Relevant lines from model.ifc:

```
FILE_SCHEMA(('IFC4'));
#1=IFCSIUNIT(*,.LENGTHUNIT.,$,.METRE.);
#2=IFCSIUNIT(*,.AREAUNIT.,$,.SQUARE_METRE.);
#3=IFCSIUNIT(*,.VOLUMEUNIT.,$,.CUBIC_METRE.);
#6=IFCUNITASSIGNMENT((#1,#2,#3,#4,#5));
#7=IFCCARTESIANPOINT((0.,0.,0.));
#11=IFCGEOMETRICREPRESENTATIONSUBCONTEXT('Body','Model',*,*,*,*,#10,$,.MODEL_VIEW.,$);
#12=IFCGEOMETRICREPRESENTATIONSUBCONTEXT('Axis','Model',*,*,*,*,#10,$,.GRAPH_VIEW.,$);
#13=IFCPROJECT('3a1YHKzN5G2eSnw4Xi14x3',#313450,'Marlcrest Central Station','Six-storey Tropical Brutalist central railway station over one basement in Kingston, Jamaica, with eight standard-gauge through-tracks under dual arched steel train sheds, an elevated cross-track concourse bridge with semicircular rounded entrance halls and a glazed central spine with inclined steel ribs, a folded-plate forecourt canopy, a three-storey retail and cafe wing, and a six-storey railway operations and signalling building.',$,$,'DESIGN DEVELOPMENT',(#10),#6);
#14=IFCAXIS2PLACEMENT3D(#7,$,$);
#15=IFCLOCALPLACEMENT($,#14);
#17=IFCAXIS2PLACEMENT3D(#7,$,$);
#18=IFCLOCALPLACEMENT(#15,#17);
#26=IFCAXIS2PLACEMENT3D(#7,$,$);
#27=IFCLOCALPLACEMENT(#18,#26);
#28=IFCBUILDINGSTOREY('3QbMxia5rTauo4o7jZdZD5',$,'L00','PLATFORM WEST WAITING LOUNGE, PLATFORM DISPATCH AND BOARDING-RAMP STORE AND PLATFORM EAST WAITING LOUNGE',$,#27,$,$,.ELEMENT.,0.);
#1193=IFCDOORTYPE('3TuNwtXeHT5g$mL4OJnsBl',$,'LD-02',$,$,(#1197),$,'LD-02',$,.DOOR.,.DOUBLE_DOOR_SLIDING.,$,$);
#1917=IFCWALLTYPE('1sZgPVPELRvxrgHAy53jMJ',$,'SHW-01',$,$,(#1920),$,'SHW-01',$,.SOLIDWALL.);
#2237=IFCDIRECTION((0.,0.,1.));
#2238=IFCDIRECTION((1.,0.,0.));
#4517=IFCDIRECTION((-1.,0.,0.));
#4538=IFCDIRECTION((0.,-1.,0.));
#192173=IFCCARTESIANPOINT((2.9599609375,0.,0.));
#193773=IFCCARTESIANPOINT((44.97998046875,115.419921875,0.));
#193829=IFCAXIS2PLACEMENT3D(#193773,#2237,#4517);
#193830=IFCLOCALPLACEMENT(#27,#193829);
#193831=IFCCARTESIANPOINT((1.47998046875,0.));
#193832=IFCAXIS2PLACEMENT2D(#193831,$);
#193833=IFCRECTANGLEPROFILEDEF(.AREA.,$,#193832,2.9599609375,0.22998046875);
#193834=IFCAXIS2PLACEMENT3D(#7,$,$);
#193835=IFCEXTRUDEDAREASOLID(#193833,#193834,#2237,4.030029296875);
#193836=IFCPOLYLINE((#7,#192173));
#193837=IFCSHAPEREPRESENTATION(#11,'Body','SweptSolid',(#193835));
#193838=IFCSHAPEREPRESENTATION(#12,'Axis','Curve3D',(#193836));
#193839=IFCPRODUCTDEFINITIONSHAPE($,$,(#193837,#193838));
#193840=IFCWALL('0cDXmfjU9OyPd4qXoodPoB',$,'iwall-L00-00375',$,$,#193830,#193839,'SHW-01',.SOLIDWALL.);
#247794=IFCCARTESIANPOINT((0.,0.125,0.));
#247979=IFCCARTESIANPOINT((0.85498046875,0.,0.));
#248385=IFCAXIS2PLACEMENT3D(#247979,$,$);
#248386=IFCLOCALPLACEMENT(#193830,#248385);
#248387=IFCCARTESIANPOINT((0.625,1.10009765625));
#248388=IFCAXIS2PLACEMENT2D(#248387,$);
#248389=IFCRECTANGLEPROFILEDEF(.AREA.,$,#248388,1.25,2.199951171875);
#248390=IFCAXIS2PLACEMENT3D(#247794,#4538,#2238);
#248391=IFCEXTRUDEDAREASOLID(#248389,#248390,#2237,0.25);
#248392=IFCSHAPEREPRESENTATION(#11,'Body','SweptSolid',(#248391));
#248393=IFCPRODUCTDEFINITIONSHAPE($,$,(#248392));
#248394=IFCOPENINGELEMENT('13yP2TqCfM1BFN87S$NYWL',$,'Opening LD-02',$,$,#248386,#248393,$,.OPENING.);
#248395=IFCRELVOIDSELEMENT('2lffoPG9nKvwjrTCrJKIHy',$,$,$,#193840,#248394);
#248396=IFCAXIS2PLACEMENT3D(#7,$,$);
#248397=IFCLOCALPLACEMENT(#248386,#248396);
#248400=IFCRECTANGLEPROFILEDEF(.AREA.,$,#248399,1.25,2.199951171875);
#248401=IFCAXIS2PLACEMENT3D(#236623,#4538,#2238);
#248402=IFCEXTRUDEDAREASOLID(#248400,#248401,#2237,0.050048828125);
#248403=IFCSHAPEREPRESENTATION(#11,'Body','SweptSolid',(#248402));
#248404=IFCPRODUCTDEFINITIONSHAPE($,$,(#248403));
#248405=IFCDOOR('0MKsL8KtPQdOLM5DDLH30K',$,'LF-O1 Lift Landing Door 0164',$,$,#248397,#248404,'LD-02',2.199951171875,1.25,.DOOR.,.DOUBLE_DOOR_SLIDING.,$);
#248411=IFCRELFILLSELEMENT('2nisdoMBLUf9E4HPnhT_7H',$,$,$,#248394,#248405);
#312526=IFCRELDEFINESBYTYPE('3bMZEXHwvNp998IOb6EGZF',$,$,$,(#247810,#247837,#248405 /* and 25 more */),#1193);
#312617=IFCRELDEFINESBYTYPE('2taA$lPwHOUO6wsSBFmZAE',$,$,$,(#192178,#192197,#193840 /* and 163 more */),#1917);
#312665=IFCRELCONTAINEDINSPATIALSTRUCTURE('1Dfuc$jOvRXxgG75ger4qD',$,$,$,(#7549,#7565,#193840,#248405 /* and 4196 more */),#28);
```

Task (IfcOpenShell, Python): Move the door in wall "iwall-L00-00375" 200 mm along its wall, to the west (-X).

```python
import ifcopenshell
import ifcopenshell.api.geometry
import ifcopenshell.util.placement
import ifcopenshell.util.unit

model = ifcopenshell.open("model.ifc")
unit_scale = ifcopenshell.util.unit.calculate_unit_scale(model)

door = model.by_guid("0MKsL8KtPQdOLM5DDLH30K")
opening = door.FillsVoids[0].RelatingOpeningElement
wall = opening.VoidsElements[0].RelatingBuildingElement

wall_matrix = ifcopenshell.util.placement.get_local_placement(wall.ObjectPlacement)
shift = wall_matrix[:3, 0] * 0.2 / unit_scale
before = ifcopenshell.util.placement.get_local_placement(door.ObjectPlacement)[:3, 3].copy()

# The door is placed relative to its opening, so it follows when the opening moves.
matrix = ifcopenshell.util.placement.get_local_placement(opening.ObjectPlacement)
matrix[:3, 3] += shift
ifcopenshell.api.geometry.edit_object_placement(
    model, product=opening, matrix=matrix, is_si=False, should_transform_children=True
)

after = ifcopenshell.util.placement.get_local_placement(door.ObjectPlacement)[:3, 3]
print("door moved by", (after - before).round(3) + 0.0)

model.write("model-out.ifc")
```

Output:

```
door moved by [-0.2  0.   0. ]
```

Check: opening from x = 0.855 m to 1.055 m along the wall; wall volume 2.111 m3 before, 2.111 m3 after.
